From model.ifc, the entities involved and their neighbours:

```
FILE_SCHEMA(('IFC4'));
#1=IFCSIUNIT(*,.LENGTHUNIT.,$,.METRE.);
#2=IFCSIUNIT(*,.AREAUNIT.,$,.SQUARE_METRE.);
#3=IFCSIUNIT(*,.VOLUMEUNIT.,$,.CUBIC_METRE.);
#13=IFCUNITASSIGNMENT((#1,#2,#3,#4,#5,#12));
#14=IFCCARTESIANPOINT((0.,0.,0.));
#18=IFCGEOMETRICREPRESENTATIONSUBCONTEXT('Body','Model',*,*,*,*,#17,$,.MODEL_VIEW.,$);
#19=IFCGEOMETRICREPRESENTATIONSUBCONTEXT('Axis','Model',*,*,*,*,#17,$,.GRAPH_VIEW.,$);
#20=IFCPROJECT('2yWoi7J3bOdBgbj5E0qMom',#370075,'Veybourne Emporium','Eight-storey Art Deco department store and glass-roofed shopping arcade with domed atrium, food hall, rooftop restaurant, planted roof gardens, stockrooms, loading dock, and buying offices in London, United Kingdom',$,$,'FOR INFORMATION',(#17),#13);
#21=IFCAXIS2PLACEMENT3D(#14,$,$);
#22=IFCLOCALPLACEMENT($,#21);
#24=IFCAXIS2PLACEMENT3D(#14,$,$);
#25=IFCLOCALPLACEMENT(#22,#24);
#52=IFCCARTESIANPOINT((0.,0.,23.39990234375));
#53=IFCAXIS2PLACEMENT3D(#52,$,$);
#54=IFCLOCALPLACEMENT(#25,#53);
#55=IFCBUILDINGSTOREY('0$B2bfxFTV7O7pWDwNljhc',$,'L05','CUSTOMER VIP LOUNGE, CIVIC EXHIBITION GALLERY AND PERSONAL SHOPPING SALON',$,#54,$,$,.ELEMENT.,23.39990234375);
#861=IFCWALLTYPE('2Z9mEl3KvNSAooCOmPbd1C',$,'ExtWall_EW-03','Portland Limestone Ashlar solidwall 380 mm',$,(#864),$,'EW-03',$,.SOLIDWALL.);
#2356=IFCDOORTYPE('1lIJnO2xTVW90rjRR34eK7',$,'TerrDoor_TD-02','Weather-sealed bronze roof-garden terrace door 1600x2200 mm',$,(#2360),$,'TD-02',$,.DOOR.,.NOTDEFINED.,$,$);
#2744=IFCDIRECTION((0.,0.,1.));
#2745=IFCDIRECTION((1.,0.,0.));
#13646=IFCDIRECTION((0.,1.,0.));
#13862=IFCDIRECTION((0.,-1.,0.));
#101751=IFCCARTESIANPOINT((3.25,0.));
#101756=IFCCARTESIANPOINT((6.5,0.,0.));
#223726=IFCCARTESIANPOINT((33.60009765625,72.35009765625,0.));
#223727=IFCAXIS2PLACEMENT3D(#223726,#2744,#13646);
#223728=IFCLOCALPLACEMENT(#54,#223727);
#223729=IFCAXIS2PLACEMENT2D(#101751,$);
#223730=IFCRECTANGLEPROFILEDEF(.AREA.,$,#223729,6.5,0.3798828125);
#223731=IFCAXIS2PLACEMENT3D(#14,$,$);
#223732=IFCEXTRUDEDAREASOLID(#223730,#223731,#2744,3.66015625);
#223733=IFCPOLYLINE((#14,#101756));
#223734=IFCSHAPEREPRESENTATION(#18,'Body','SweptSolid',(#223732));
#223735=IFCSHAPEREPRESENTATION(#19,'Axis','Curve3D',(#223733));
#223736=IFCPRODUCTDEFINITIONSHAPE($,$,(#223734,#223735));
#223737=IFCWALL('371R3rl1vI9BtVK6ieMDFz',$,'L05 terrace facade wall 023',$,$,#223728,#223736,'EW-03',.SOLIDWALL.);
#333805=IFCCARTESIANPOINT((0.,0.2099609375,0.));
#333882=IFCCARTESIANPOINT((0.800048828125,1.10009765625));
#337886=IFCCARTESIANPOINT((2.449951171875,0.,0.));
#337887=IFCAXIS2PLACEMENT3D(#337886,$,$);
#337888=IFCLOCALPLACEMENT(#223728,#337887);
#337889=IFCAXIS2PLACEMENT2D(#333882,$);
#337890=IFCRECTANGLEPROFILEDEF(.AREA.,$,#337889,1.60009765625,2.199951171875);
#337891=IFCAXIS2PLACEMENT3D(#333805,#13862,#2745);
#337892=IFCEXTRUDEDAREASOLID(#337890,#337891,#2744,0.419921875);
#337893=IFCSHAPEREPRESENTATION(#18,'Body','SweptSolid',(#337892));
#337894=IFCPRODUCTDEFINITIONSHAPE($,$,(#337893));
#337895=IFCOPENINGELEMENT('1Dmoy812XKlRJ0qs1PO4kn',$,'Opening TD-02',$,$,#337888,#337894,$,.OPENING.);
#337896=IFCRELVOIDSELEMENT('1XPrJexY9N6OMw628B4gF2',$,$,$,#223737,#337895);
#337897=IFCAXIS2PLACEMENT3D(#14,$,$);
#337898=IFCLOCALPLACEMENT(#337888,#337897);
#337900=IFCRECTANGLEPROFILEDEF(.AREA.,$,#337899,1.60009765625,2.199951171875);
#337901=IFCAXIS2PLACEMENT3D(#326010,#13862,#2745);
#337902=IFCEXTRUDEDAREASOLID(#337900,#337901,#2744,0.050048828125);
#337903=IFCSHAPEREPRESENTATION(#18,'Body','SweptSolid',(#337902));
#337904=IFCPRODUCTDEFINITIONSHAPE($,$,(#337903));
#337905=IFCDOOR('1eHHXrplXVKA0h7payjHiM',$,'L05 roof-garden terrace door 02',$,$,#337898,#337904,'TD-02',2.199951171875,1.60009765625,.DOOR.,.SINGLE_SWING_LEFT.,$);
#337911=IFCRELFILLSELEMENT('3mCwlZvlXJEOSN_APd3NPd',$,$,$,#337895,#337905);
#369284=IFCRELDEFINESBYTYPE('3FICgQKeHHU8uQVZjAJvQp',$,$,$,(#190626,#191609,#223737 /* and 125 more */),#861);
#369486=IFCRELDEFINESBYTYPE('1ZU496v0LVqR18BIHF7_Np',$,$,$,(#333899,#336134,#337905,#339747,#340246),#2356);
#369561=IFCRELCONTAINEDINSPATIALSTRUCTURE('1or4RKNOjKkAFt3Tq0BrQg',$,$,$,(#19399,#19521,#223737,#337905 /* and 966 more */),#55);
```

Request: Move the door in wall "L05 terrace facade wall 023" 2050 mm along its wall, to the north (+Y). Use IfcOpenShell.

```python
import ifcopenshell
import ifcopenshell.api.geometry
import ifcopenshell.util.placement
import ifcopenshell.util.unit

model = ifcopenshell.open("model.ifc")
unit_scale = ifcopenshell.util.unit.calculate_unit_scale(model)

door = model.by_guid("1eHHXrplXVKA0h7payjHiM")
opening = door.FillsVoids[0].RelatingOpeningElement
wall = opening.VoidsElements[0].RelatingBuildingElement

wall_matrix = ifcopenshell.util.placement.get_local_placement(wall.ObjectPlacement)
shift = wall_matrix[:3, 0] * 2.05 / unit_scale
before = ifcopenshell.util.placement.get_local_placement(door.ObjectPlacement)[:3, 3].copy()

# The door is placed relative to its opening, so it follows when the opening moves.
matrix = ifcopenshell.util.placement.get_local_placement(opening.ObjectPlacement)
matrix[:3, 3] += shift
ifcopenshell.api.geometry.edit_object_placement(
    model, product=opening, matrix=matrix, is_si=False, should_transform_children=True
)

after = ifcopenshell.util.placement.get_local_placement(door.ObjectPlacement)[:3, 3]
print("door moved by", (after - before).round(3) + 0.0)

model.write("model_edited.ifc")
```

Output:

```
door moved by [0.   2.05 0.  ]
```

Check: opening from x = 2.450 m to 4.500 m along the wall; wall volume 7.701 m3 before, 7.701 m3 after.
